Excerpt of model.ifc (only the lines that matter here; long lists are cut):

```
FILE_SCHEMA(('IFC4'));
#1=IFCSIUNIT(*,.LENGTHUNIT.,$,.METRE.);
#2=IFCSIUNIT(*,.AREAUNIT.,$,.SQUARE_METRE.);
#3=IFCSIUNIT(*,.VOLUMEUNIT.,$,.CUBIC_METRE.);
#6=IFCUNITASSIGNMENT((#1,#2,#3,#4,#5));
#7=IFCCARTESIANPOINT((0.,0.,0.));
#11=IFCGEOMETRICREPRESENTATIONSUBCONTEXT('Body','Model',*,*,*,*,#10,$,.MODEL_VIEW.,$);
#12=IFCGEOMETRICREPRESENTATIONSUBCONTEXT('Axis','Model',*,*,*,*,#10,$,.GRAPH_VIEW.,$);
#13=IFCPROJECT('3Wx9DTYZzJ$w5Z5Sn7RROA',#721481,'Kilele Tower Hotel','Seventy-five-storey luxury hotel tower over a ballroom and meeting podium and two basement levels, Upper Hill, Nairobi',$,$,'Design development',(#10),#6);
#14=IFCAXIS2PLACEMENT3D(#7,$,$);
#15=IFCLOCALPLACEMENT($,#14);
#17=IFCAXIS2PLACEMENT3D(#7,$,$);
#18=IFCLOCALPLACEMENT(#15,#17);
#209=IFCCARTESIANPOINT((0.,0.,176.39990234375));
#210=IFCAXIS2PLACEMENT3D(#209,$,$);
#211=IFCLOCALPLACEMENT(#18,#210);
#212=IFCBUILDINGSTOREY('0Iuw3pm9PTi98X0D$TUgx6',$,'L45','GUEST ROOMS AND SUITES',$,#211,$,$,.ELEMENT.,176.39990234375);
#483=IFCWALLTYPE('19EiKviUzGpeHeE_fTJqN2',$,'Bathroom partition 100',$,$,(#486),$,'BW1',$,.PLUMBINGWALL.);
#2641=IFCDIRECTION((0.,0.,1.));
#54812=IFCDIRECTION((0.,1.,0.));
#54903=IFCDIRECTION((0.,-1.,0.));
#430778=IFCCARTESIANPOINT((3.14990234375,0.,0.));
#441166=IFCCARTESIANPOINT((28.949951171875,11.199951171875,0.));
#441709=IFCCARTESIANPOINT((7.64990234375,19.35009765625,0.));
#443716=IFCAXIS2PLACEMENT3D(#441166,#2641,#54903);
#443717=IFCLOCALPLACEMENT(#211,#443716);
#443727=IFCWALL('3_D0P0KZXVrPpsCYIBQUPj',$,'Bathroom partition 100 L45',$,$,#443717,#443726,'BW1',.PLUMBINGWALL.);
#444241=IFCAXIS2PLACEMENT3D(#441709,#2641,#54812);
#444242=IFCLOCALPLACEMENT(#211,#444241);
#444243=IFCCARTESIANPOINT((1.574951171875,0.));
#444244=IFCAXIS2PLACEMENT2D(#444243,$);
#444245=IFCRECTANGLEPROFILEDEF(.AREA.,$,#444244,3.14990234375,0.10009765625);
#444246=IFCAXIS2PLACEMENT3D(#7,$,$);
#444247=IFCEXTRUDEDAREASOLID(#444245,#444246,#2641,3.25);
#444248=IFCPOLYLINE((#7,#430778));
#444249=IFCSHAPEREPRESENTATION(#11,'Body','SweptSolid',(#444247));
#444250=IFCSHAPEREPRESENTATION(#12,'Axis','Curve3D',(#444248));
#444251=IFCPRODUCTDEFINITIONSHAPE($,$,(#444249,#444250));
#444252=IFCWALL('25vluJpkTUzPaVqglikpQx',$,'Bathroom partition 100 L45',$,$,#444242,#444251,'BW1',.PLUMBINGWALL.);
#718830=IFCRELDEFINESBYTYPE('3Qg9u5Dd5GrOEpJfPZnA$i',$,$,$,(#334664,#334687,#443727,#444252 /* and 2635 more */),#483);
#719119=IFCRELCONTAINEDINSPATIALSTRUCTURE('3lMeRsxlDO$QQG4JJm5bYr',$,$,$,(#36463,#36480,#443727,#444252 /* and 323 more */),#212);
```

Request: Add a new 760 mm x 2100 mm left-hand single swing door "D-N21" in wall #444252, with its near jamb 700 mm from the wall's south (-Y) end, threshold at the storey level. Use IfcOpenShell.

```python
import numpy as np
import ifcopenshell
import ifcopenshell.api.feature
import ifcopenshell.api.geometry
import ifcopenshell.api.root
import ifcopenshell.api.spatial
import ifcopenshell.geom
import ifcopenshell.util.element
import ifcopenshell.util.placement
import ifcopenshell.util.representation
import ifcopenshell.util.shape
import ifcopenshell.util.unit

model = ifcopenshell.open("model.ifc")
unit_scale = ifcopenshell.util.unit.calculate_unit_scale(model)
settings = ifcopenshell.geom.settings()


def volume(element):
    """Net volume in cubic metres, openings subtracted."""
    shape = ifcopenshell.geom.create_shape(settings, element)
    return ifcopenshell.util.shape.get_volume(shape.geometry)


wall = model.by_guid("25vluJpkTUzPaVqglikpQx")
storey = ifcopenshell.util.element.get_container(wall, ifc_class="IfcBuildingStorey")
context = ifcopenshell.util.representation.get_context(model, "Model", "Body", "MODEL_VIEW")
before = volume(wall)

width, height, from_end, sill = 0.76, 2.1, 0.7, 0.0  # metres

# The wall runs along its own X axis, and the end named is its -X end.
wall_shape = ifcopenshell.geom.create_shape(settings, wall)
x, y, z = ifcopenshell.util.shape.get_vertices(wall_shape.geometry).T
start = x.min() + from_end
face, thickness = float(y.min()), float(y.max() - y.min())
wall_matrix = ifcopenshell.util.placement.get_local_placement(wall.ObjectPlacement)
level = ifcopenshell.util.placement.get_local_placement(storey.ObjectPlacement)[2, 3]


def in_wall(x, y):
    """Placement at x, y metres in the wall's axes, at sill height."""
    matrix = wall_matrix.copy()
    matrix[:, 3] = wall_matrix @ np.array([x / unit_scale, y / unit_scale, 0.0, 1.0])
    matrix[2, 3] = level + sill / unit_scale
    return matrix


# Opening: a box that overshoots both wall faces by 50 mm.
opening = ifcopenshell.api.root.create_entity(model, ifc_class="IfcOpeningElement", predefined_type="OPENING")
box = ifcopenshell.api.geometry.add_wall_representation(
    model, context=context, length=width, height=height, thickness=thickness + 0.1
)
ifcopenshell.api.geometry.assign_representation(model, product=opening, representation=box)
ifcopenshell.api.geometry.edit_object_placement(model, product=opening, matrix=in_wall(start, face - 0.05), is_si=False)
ifcopenshell.api.feature.add_feature(model, feature=opening, element=wall)

door = ifcopenshell.api.root.create_entity(model, ifc_class="IfcDoor", name="D-N21", predefined_type="DOOR")
door.OverallWidth, door.OverallHeight = width / unit_scale, height / unit_scale
door.OperationType = "SINGLE_SWING_LEFT"
body = ifcopenshell.api.geometry.add_door_representation(
    model,
    context=context,
    overall_width=door.OverallWidth,
    overall_height=door.OverallHeight,
    operation_type="SINGLE_SWING_LEFT",
    lining_properties={"LiningDepth": thickness / unit_scale, "ThresholdDepth": thickness / unit_scale},
)
ifcopenshell.api.geometry.assign_representation(model, product=door, representation=body)
ifcopenshell.api.spatial.assign_container(model, products=[door], relating_structure=storey)
ifcopenshell.api.feature.add_filling(model, opening=opening, element=door)

# The lining spans the wall, so the door starts at the wall face.
ifcopenshell.api.geometry.edit_object_placement(model, product=door, matrix=in_wall(start, face), is_si=False)

after = volume(wall)

print(f"wall volume {before:.3f} -> {after:.3f} m3")

model.write("model-out.ifc")
```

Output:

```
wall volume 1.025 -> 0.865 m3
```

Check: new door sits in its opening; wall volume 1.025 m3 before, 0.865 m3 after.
